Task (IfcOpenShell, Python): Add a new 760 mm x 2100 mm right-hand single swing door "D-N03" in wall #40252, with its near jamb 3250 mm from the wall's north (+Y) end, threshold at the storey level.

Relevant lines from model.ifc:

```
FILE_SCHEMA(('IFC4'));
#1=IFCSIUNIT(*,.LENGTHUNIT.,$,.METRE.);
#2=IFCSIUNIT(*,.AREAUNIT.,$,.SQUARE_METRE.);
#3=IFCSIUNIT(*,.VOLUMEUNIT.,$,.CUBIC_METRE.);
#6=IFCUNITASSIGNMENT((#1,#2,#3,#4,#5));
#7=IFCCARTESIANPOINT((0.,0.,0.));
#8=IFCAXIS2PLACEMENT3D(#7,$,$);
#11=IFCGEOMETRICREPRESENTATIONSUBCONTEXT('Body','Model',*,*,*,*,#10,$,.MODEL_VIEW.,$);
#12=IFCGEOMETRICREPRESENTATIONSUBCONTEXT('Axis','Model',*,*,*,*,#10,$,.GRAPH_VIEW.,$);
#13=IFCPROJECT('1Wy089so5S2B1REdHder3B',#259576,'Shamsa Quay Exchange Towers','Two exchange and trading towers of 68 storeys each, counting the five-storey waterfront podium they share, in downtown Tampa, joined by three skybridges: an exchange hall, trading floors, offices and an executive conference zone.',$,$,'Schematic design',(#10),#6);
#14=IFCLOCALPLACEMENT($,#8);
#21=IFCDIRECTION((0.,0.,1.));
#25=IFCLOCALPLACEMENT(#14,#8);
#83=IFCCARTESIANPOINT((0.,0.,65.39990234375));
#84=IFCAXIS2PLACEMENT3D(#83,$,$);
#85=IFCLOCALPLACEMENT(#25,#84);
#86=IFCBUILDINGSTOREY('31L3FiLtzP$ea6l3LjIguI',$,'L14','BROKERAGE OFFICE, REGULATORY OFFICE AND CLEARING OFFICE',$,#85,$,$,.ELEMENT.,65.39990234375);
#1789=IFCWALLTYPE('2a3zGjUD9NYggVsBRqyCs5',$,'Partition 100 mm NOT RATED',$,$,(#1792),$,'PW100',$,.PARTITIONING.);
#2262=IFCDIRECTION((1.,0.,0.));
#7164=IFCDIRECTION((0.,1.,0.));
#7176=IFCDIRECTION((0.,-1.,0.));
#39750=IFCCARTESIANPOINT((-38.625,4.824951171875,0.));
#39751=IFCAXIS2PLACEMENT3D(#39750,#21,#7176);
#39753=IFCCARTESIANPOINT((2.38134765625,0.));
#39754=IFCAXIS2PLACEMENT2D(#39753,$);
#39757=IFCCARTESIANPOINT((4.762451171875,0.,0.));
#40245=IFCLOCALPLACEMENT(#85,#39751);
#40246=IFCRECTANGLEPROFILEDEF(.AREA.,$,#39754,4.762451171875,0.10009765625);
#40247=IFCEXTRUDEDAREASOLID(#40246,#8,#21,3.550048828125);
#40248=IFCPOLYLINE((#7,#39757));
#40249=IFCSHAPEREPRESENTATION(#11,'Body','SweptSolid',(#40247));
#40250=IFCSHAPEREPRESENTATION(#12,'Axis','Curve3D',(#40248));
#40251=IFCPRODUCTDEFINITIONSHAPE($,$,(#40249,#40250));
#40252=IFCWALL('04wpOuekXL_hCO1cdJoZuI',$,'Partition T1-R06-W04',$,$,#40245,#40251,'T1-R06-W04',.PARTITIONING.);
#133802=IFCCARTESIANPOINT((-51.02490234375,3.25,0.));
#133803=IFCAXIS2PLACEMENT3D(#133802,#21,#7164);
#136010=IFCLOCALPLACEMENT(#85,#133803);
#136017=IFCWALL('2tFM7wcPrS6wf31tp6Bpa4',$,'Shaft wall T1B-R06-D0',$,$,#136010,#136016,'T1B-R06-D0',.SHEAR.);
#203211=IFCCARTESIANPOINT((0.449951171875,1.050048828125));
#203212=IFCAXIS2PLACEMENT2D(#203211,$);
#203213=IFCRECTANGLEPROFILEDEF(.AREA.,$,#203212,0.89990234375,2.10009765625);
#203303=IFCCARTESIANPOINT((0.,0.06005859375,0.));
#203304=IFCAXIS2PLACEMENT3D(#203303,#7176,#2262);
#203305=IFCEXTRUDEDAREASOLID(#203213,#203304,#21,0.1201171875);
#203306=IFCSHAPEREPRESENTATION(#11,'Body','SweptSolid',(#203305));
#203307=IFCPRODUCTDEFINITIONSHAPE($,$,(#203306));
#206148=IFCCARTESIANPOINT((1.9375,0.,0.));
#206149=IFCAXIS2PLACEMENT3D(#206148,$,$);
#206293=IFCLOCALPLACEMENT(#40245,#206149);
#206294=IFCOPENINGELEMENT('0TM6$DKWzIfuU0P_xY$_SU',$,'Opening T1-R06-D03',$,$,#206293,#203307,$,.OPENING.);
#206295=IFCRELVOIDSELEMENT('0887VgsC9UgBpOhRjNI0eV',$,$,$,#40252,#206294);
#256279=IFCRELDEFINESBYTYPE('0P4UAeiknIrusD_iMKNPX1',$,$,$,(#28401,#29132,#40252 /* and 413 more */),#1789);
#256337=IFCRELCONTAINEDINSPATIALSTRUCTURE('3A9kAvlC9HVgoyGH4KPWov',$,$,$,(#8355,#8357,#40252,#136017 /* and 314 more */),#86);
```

```python
import numpy as np
import ifcopenshell
import ifcopenshell.api.feature
import ifcopenshell.api.geometry
import ifcopenshell.api.root
import ifcopenshell.api.spatial
import ifcopenshell.geom
import ifcopenshell.util.element
import ifcopenshell.util.placement
import ifcopenshell.util.representation
import ifcopenshell.util.shape
import ifcopenshell.util.unit

model = ifcopenshell.open("model.ifc")
unit_scale = ifcopenshell.util.unit.calculate_unit_scale(model)
settings = ifcopenshell.geom.settings()


def volume(element):
    """Net volume in cubic metres, openings subtracted."""
    shape = ifcopenshell.geom.create_shape(settings, element)
    return ifcopenshell.util.shape.get_volume(shape.geometry)


wall = model.by_guid("04wpOuekXL_hCO1cdJoZuI")
storey = ifcopenshell.util.element.get_container(wall, ifc_class="IfcBuildingStorey")
context = ifcopenshell.util.representation.get_context(model, "Model", "Body", "MODEL_VIEW")
before = volume(wall)

width, height, from_end, sill = 0.76, 2.1, 3.25, 0.0  # metres

# The wall runs along its own X axis, and the end named is its -X end.
wall_shape = ifcopenshell.geom.create_shape(settings, wall)
x, y, z = ifcopenshell.util.shape.get_vertices(wall_shape.geometry).T
start = x.min() + from_end
face, thickness = float(y.min()), float(y.max() - y.min())
wall_matrix = ifcopenshell.util.placement.get_local_placement(wall.ObjectPlacement)
level = ifcopenshell.util.placement.get_local_placement(storey.ObjectPlacement)[2, 3]


def in_wall(x, y):
    """Placement at x, y metres in the wall's axes, at sill height."""
    matrix = wall_matrix.copy()
    matrix[:, 3] = wall_matrix @ np.array([x / unit_scale, y / unit_scale, 0.0, 1.0])
    matrix[2, 3] = level + sill / unit_scale
    return matrix


# Opening: a box that overshoots both wall faces by 50 mm.
opening = ifcopenshell.api.root.create_entity(model, ifc_class="IfcOpeningElement", predefined_type="OPENING")
box = ifcopenshell.api.geometry.add_wall_representation(
    model, context=context, length=width, height=height, thickness=thickness + 0.1
)
ifcopenshell.api.geometry.assign_representation(model, product=opening, representation=box)
ifcopenshell.api.geometry.edit_object_placement(model, product=opening, matrix=in_wall(start, face - 0.05), is_si=False)
ifcopenshell.api.feature.add_feature(model, feature=opening, element=wall)

door = ifcopenshell.api.root.create_entity(model, ifc_class="IfcDoor", name="D-N03", predefined_type="DOOR")
door.OverallWidth, door.OverallHeight = width / unit_scale, height / unit_scale
door.OperationType = "SINGLE_SWING_RIGHT"
body = ifcopenshell.api.geometry.add_door_representation(
    model,
    context=context,
    overall_width=door.OverallWidth,
    overall_height=door.OverallHeight,
    operation_type="SINGLE_SWING_RIGHT",
    lining_properties={"LiningDepth": thickness / unit_scale, "ThresholdDepth": thickness / unit_scale},
)
ifcopenshell.api.geometry.assign_representation(model, product=door, representation=body)
ifcopenshell.api.spatial.assign_container(model, products=[door], relating_structure=storey)
ifcopenshell.api.feature.add_filling(model, opening=opening, element=door)

# The lining spans the wall, so the door starts at the wall face.
ifcopenshell.api.geometry.edit_object_placement(model, product=door, matrix=in_wall(start, face), is_si=False)

after = volume(wall)

print(f"wall volume {before:.3f} -> {after:.3f} m3")

model.write("model_updated.ifc")
```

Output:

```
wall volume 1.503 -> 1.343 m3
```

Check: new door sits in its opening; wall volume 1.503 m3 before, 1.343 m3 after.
